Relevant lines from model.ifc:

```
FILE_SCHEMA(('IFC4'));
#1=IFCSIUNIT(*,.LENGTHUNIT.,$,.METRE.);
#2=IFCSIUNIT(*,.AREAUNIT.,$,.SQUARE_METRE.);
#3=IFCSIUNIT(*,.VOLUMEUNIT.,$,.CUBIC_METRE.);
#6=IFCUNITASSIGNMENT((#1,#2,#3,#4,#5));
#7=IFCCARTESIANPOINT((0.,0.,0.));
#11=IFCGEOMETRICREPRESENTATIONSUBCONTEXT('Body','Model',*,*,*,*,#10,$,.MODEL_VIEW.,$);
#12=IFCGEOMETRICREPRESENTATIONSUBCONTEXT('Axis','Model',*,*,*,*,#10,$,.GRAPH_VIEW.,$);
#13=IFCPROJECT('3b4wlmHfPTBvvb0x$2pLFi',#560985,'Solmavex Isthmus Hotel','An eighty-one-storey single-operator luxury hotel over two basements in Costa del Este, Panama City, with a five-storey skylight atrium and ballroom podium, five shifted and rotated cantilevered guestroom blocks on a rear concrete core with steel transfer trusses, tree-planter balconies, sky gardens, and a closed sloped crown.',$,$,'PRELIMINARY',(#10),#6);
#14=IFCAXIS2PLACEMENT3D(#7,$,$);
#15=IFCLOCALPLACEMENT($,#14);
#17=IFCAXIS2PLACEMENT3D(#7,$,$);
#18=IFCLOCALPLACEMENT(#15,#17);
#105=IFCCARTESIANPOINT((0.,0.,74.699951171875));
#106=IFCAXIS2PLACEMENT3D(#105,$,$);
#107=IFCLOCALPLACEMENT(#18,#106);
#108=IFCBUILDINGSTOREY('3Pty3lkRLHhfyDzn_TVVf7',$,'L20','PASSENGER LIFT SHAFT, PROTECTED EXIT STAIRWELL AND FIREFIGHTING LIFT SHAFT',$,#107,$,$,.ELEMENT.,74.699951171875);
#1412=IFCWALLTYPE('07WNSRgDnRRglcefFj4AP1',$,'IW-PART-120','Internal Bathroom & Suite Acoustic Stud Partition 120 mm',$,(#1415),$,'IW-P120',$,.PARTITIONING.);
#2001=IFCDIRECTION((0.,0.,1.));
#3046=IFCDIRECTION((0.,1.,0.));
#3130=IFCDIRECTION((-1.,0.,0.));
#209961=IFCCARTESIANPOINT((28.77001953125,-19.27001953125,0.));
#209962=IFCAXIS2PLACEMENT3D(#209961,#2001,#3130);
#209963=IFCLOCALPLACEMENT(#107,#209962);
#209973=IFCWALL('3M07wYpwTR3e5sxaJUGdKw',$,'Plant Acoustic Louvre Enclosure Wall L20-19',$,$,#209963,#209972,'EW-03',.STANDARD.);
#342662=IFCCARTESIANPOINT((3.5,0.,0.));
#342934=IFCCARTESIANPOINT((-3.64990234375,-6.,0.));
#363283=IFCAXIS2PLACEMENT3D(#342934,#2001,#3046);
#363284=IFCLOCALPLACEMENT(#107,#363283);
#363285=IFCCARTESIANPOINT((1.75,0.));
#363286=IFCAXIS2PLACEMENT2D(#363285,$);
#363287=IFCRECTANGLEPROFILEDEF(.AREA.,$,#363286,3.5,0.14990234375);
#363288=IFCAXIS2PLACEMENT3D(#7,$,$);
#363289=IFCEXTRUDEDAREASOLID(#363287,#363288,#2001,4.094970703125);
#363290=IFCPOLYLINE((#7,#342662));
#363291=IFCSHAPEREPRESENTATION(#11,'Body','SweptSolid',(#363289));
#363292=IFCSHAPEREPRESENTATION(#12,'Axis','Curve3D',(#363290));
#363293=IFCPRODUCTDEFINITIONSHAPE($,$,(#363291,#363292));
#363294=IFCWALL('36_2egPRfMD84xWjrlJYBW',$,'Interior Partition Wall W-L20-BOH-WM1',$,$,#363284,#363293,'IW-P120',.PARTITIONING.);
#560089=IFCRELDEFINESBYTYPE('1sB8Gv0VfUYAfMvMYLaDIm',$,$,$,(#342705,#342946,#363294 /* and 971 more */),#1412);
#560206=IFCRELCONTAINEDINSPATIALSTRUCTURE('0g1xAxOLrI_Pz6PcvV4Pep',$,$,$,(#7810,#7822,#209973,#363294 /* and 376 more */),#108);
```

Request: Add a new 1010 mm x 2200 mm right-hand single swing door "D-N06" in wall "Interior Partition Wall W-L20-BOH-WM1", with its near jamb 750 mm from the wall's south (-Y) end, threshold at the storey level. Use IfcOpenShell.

```python
import numpy as np
import ifcopenshell
import ifcopenshell.api.feature
import ifcopenshell.api.geometry
import ifcopenshell.api.root
import ifcopenshell.api.spatial
import ifcopenshell.geom
import ifcopenshell.util.element
import ifcopenshell.util.placement
import ifcopenshell.util.representation
import ifcopenshell.util.shape
import ifcopenshell.util.unit

model = ifcopenshell.open("model.ifc")
unit_scale = ifcopenshell.util.unit.calculate_unit_scale(model)
settings = ifcopenshell.geom.settings()


def volume(element):
    """Net volume in cubic metres, openings subtracted."""
    shape = ifcopenshell.geom.create_shape(settings, element)
    return ifcopenshell.util.shape.get_volume(shape.geometry)


wall = model.by_guid("36_2egPRfMD84xWjrlJYBW")
storey = ifcopenshell.util.element.get_container(wall, ifc_class="IfcBuildingStorey")
context = ifcopenshell.util.representation.get_context(model, "Model", "Body", "MODEL_VIEW")
before = volume(wall)

width, height, from_end, sill = 1.01, 2.2, 0.75, 0.0  # metres

# The wall runs along its own X axis, and the end named is its -X end.
wall_shape = ifcopenshell.geom.create_shape(settings, wall)
x, y, z = ifcopenshell.util.shape.get_vertices(wall_shape.geometry).T
start = x.min() + from_end
face, thickness = float(y.min()), float(y.max() - y.min())
wall_matrix = ifcopenshell.util.placement.get_local_placement(wall.ObjectPlacement)
level = ifcopenshell.util.placement.get_local_placement(storey.ObjectPlacement)[2, 3]


def in_wall(x, y):
    """Placement at x, y metres in the wall's axes, at sill height."""
    matrix = wall_matrix.copy()
    matrix[:, 3] = wall_matrix @ np.array([x / unit_scale, y / unit_scale, 0.0, 1.0])
    matrix[2, 3] = level + sill / unit_scale
    return matrix


# Opening: a box that overshoots both wall faces by 50 mm.
opening = ifcopenshell.api.root.create_entity(model, ifc_class="IfcOpeningElement", predefined_type="OPENING")
box = ifcopenshell.api.geometry.add_wall_representation(
    model, context=context, length=width, height=height, thickness=thickness + 0.1
)
ifcopenshell.api.geometry.assign_representation(model, product=opening, representation=box)
ifcopenshell.api.geometry.edit_object_placement(model, product=opening, matrix=in_wall(start, face - 0.05), is_si=False)
ifcopenshell.api.feature.add_feature(model, feature=opening, element=wall)

door = ifcopenshell.api.root.create_entity(model, ifc_class="IfcDoor", name="D-N06", predefined_type="DOOR")
door.OverallWidth, door.OverallHeight = width / unit_scale, height / unit_scale
door.OperationType = "SINGLE_SWING_RIGHT"
body = ifcopenshell.api.geometry.add_door_representation(
    model,
    context=context,
    overall_width=door.OverallWidth,
    overall_height=door.OverallHeight,
    operation_type="SINGLE_SWING_RIGHT",
    lining_properties={"LiningDepth": thickness / unit_scale, "ThresholdDepth": thickness / unit_scale},
)
ifcopenshell.api.geometry.assign_representation(model, product=door, representation=body)
ifcopenshell.api.spatial.assign_container(model, products=[door], relating_structure=storey)
ifcopenshell.api.feature.add_filling(model, opening=opening, element=door)

# The lining spans the wall, so the door starts at the wall face.
ifcopenshell.api.geometry.edit_object_placement(model, product=door, matrix=in_wall(start, face), is_si=False)

after = volume(wall)

print(f"wall volume {before:.3f} -> {after:.3f} m3")

model.write("model_v2.ifc")
```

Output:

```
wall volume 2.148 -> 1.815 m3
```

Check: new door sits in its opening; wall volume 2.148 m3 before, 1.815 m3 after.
